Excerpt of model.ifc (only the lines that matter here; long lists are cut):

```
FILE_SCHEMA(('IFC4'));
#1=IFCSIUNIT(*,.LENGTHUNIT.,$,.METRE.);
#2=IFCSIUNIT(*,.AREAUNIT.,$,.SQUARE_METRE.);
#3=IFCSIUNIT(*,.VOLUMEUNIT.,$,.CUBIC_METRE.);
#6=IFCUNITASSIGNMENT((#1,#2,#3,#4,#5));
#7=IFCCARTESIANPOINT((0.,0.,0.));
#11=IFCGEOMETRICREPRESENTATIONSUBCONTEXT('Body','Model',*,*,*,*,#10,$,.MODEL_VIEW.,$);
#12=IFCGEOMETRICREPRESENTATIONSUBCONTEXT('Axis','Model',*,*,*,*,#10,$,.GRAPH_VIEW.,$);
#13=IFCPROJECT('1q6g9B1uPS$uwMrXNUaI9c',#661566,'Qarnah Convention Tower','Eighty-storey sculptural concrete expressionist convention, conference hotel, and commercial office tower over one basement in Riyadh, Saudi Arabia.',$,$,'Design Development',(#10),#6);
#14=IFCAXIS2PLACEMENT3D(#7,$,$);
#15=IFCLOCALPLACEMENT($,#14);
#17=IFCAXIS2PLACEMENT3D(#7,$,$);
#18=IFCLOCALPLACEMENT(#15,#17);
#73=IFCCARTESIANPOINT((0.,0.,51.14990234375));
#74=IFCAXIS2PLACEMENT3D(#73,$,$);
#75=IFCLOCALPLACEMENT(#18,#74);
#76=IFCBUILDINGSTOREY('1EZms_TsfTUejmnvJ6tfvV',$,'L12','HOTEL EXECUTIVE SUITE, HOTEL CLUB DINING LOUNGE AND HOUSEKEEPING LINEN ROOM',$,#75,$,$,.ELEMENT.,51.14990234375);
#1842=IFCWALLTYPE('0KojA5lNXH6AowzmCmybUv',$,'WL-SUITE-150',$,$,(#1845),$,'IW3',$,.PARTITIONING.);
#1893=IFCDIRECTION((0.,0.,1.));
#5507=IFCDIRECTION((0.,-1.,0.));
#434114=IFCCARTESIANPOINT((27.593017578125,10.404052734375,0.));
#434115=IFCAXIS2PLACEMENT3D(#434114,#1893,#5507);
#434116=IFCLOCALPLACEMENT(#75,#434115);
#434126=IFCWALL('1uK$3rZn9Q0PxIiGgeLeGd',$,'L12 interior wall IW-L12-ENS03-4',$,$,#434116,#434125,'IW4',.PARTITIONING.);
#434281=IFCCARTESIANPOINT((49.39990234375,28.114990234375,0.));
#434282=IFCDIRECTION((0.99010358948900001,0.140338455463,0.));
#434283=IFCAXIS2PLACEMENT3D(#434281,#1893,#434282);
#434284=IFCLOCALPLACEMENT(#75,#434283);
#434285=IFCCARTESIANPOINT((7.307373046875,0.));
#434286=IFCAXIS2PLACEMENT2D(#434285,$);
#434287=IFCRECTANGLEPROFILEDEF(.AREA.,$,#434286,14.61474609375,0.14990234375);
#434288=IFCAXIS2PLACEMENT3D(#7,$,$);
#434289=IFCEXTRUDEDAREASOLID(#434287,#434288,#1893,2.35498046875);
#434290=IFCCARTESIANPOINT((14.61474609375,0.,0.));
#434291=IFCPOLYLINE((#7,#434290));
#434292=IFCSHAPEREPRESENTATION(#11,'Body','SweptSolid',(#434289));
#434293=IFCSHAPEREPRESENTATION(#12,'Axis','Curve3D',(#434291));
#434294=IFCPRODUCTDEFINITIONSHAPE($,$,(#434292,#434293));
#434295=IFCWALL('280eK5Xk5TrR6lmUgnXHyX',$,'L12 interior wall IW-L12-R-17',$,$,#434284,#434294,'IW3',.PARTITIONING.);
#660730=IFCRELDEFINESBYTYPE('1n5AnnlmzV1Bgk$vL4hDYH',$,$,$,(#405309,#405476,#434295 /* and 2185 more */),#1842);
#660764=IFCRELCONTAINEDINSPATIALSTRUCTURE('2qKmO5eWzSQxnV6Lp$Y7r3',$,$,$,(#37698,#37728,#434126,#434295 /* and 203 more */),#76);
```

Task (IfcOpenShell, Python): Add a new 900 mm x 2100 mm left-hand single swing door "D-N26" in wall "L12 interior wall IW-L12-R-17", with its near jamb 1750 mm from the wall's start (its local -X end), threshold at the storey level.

```python
import numpy as np
import ifcopenshell
import ifcopenshell.api.feature
import ifcopenshell.api.geometry
import ifcopenshell.api.root
import ifcopenshell.api.spatial
import ifcopenshell.geom
import ifcopenshell.util.element
import ifcopenshell.util.placement
import ifcopenshell.util.representation
import ifcopenshell.util.shape
import ifcopenshell.util.unit

model = ifcopenshell.open("model.ifc")
unit_scale = ifcopenshell.util.unit.calculate_unit_scale(model)
settings = ifcopenshell.geom.settings()


def volume(element):
    """Net volume in cubic metres, openings subtracted."""
    shape = ifcopenshell.geom.create_shape(settings, element)
    return ifcopenshell.util.shape.get_volume(shape.geometry)


wall = model.by_id(434295)
storey = ifcopenshell.util.element.get_container(wall, ifc_class="IfcBuildingStorey")
context = ifcopenshell.util.representation.get_context(model, "Model", "Body", "MODEL_VIEW")
before = volume(wall)

width, height, from_end, sill = 0.9, 2.1, 1.75, 0.0  # metres

# The wall runs along its own X axis, and the end named is its -X end.
wall_shape = ifcopenshell.geom.create_shape(settings, wall)
x, y, z = ifcopenshell.util.shape.get_vertices(wall_shape.geometry).T
start = x.min() + from_end
face, thickness = float(y.min()), float(y.max() - y.min())
wall_matrix = ifcopenshell.util.placement.get_local_placement(wall.ObjectPlacement)
level = ifcopenshell.util.placement.get_local_placement(storey.ObjectPlacement)[2, 3]


def in_wall(x, y):
    """Placement at x, y metres in the wall's axes, at sill height."""
    matrix = wall_matrix.copy()
    matrix[:, 3] = wall_matrix @ np.array([x / unit_scale, y / unit_scale, 0.0, 1.0])
    matrix[2, 3] = level + sill / unit_scale
    return matrix


# Opening: a box that overshoots both wall faces by 50 mm.
opening = ifcopenshell.api.root.create_entity(model, ifc_class="IfcOpeningElement", predefined_type="OPENING")
box = ifcopenshell.api.geometry.add_wall_representation(
    model, context=context, length=width, height=height, thickness=thickness + 0.1
)
ifcopenshell.api.geometry.assign_representation(model, product=opening, representation=box)
ifcopenshell.api.geometry.edit_object_placement(model, product=opening, matrix=in_wall(start, face - 0.05), is_si=False)
ifcopenshell.api.feature.add_feature(model, feature=opening, element=wall)

door = ifcopenshell.api.root.create_entity(model, ifc_class="IfcDoor", name="D-N26", predefined_type="DOOR")
door.OverallWidth, door.OverallHeight = width / unit_scale, height / unit_scale
door.OperationType = "SINGLE_SWING_LEFT"
body = ifcopenshell.api.geometry.add_door_representation(
    model,
    context=context,
    overall_width=door.OverallWidth,
    overall_height=door.OverallHeight,
    operation_type="SINGLE_SWING_LEFT",
    lining_properties={"LiningDepth": thickness / unit_scale, "ThresholdDepth": thickness / unit_scale},
)
ifcopenshell.api.geometry.assign_representation(model, product=door, representation=body)
ifcopenshell.api.spatial.assign_container(model, products=[door], relating_structure=storey)
ifcopenshell.api.feature.add_filling(model, opening=opening, element=door)

# The lining spans the wall, so the door starts at the wall face.
ifcopenshell.api.geometry.edit_object_placement(model, product=door, matrix=in_wall(start, face), is_si=False)

after = volume(wall)

print(f"wall volume {before:.3f} -> {after:.3f} m3")

model.write("model_edited.ifc")
```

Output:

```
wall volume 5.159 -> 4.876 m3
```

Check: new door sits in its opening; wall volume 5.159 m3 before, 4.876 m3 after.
